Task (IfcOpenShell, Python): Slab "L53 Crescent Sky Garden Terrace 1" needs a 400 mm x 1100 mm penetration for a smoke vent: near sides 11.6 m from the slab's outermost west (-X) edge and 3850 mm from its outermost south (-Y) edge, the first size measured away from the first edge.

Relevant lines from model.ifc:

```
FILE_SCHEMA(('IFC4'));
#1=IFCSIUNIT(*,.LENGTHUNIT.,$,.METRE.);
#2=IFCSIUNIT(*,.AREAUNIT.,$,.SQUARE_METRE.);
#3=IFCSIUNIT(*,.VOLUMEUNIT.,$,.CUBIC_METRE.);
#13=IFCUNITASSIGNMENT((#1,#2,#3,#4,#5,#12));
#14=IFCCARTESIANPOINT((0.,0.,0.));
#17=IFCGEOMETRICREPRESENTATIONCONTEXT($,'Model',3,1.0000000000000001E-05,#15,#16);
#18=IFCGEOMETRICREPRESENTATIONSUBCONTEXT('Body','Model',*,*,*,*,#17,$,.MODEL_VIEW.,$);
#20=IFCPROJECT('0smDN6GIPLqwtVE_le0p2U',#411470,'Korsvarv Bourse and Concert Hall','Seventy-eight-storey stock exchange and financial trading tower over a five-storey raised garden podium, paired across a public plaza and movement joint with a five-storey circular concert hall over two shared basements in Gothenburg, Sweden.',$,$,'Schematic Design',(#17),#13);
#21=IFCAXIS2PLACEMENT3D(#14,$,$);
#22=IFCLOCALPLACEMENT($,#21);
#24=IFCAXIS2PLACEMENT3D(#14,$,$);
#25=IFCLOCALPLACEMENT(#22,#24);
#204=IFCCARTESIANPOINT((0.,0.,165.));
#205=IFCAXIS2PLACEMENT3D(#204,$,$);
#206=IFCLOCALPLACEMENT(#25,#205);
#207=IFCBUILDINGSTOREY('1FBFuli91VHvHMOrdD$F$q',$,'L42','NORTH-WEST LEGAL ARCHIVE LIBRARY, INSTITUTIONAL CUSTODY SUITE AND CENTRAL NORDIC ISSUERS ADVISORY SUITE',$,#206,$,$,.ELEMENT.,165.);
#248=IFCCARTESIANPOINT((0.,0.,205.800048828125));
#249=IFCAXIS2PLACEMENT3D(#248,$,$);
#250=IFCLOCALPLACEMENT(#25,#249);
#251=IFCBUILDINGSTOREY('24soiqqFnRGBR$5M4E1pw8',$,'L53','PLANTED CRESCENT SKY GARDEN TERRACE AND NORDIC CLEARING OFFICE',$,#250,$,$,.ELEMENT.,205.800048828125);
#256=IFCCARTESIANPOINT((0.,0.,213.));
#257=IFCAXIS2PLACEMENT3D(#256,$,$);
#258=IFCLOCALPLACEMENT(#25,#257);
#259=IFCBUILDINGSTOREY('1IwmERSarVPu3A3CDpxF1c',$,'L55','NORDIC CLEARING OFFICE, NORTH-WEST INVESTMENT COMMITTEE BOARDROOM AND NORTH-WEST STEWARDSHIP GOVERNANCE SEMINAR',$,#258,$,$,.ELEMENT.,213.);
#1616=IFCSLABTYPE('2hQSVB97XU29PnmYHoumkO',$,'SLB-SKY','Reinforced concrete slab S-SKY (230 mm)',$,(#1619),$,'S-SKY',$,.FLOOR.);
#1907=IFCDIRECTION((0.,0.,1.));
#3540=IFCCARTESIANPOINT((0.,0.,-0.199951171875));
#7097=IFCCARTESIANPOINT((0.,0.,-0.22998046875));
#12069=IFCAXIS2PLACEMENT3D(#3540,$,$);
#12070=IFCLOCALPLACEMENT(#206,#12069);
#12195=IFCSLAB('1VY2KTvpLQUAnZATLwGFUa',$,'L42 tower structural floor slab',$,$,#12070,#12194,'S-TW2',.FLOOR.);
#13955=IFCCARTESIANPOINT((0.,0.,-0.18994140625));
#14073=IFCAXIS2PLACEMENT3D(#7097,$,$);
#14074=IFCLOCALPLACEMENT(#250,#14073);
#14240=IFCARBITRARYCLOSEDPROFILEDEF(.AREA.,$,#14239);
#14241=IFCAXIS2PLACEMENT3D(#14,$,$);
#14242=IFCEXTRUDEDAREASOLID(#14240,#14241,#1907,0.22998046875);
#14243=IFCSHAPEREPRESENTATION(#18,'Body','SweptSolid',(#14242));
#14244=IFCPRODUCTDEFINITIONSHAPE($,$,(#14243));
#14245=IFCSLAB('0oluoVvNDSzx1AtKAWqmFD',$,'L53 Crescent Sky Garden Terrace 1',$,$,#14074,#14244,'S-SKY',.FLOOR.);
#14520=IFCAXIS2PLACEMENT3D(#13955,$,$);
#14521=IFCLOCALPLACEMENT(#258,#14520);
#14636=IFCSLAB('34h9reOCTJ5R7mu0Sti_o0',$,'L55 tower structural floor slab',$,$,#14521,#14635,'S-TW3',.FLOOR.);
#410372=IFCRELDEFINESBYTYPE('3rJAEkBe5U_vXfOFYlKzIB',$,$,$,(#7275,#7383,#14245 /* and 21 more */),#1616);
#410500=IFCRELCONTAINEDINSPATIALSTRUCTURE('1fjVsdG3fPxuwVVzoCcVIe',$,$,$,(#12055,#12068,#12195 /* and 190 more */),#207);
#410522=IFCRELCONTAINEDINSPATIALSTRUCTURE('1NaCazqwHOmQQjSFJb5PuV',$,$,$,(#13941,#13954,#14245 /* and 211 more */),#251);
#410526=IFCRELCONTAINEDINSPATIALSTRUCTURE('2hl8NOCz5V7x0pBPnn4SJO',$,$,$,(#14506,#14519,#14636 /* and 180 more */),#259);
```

```python
import numpy as np
import ifcopenshell
import ifcopenshell.api.feature
import ifcopenshell.api.geometry
import ifcopenshell.api.root
import ifcopenshell.geom
import ifcopenshell.util.placement
import ifcopenshell.util.representation
import ifcopenshell.util.shape
import ifcopenshell.util.unit

model = ifcopenshell.open("model.ifc")
unit_scale = ifcopenshell.util.unit.calculate_unit_scale(model)
settings = ifcopenshell.geom.settings()


def volume(element):
    """Net volume in cubic metres, openings subtracted."""
    shape = ifcopenshell.geom.create_shape(settings, element)
    return ifcopenshell.util.shape.get_volume(shape.geometry)


slab = model.by_id(14245)
before = volume(slab)

# Extent in the slab's own axes, in metres. The edges named are its -X and -Y sides.
slab_shape = ifcopenshell.geom.create_shape(settings, slab)
vertices = ifcopenshell.util.shape.get_vertices(slab_shape.geometry)
x_min, y_min, bottom = vertices.min(axis=0)
top = vertices[:, 2].max()

opening = ifcopenshell.api.root.create_entity(model, ifc_class="IfcOpeningElement", name="Smoke vent opening", predefined_type="OPENING")
context = ifcopenshell.util.representation.get_context(model, "Model", "Body", "MODEL_VIEW")
width, depth = 0.4, 1.1
outline = [(0.0, 0.0), (width, 0.0), (width, depth), (0.0, depth), (0.0, 0.0)]
# Overshoot both faces by 50 mm so the cut is clean.
shape = ifcopenshell.api.geometry.add_slab_representation(
    model, context=context, depth=top - bottom + 0.1, polyline=outline
)
ifcopenshell.api.geometry.assign_representation(model, product=opening, representation=shape)

matrix = ifcopenshell.util.placement.get_local_placement(slab.ObjectPlacement)
matrix[:, 3] = matrix @ np.append(np.array([x_min + 11.6, y_min + 3.85, bottom - 0.05]) / unit_scale, 1.0)
ifcopenshell.api.geometry.edit_object_placement(model, product=opening, matrix=matrix, is_si=False)
ifcopenshell.api.feature.add_feature(model, feature=opening, element=slab)

after = volume(slab)

print(f"slab volume {before:.3f} -> {after:.3f} m3")

model.write("model_rev.ifc")
```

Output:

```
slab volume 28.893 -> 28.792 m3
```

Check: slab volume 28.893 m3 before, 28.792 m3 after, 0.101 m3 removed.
